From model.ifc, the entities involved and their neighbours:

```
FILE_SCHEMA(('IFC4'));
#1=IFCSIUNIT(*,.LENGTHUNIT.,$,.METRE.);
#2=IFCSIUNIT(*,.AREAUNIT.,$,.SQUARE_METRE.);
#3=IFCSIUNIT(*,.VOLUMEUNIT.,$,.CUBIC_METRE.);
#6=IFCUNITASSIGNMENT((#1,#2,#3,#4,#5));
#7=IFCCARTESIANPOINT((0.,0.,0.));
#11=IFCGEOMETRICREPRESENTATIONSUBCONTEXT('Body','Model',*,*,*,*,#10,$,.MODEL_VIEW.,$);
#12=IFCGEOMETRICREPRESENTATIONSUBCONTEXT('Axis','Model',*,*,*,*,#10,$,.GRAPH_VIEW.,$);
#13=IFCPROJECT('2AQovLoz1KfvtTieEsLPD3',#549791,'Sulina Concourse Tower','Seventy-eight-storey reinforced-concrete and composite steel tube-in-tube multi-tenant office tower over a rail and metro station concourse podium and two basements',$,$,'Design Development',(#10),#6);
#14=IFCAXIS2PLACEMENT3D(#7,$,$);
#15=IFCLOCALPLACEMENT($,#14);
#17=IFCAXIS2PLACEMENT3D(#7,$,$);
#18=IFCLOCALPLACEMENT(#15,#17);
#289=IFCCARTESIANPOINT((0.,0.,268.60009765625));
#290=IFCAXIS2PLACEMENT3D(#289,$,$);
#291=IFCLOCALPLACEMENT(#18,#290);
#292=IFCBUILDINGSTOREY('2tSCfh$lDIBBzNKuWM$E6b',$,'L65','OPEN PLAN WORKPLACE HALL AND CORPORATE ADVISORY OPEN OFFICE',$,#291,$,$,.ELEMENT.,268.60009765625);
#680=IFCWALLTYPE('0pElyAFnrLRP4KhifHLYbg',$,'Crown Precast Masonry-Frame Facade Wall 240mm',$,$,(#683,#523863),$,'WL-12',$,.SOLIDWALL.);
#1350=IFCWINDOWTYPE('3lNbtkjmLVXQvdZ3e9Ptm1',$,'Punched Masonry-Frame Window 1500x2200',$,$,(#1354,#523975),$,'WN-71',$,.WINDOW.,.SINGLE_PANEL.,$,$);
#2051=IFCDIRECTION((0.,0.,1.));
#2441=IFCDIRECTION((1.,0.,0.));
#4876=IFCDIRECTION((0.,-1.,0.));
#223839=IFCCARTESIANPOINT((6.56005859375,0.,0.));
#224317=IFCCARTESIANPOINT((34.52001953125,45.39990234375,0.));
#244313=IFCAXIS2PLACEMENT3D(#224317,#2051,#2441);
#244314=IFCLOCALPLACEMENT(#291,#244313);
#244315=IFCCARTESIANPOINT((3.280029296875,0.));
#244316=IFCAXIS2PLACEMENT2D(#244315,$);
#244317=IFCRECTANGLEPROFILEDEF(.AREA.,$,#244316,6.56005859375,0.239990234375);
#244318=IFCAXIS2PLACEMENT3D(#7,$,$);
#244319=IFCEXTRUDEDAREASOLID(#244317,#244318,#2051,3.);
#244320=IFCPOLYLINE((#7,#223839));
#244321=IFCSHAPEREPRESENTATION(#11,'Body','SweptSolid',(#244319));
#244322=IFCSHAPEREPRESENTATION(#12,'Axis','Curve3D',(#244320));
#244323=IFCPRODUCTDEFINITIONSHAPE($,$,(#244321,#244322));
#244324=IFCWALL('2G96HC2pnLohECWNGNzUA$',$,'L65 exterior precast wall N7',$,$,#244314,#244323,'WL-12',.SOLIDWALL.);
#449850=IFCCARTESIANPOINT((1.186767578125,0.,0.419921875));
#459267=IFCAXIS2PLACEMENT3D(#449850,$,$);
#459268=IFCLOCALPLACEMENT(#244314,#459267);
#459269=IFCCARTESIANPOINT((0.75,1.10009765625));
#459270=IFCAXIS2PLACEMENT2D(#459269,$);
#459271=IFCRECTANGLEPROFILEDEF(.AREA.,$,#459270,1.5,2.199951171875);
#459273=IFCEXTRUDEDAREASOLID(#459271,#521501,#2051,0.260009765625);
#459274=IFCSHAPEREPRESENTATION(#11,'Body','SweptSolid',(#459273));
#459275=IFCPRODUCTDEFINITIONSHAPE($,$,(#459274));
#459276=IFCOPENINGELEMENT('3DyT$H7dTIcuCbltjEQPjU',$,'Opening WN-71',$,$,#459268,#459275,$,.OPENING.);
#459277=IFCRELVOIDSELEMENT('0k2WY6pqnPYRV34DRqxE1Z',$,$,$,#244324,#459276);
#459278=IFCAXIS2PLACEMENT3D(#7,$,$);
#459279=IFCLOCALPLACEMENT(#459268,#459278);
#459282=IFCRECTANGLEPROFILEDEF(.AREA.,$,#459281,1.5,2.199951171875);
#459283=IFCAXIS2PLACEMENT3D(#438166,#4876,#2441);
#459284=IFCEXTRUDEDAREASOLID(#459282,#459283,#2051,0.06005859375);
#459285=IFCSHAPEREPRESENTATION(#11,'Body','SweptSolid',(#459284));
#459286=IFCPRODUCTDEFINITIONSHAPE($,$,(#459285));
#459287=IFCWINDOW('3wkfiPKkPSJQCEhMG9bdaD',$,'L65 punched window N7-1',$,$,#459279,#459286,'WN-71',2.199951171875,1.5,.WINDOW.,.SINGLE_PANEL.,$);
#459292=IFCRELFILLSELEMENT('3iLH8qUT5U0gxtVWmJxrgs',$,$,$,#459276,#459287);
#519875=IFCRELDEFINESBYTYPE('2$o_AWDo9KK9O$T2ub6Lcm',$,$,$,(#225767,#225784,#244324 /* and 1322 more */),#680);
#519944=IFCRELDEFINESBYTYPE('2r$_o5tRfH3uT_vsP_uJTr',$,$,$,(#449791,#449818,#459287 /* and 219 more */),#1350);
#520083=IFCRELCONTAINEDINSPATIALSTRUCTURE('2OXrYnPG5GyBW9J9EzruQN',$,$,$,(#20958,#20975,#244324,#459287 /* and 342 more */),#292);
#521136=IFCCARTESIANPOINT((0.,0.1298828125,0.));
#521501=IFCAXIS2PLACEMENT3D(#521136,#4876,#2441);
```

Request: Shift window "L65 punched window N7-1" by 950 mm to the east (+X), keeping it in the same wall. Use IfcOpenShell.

```python
import ifcopenshell
import ifcopenshell.api.geometry
import ifcopenshell.util.placement

model = ifcopenshell.open("model.ifc")

window = model.by_guid("3wkfiPKkPSJQCEhMG9bdaD")
opening = window.FillsVoids[0].RelatingOpeningElement
wall = opening.VoidsElements[0].RelatingBuildingElement

wall_matrix = ifcopenshell.util.placement.get_local_placement(wall.ObjectPlacement)
shift = wall_matrix[:3, 0] * 0.95
before = ifcopenshell.util.placement.get_local_placement(window.ObjectPlacement)[:3, 3].copy()

# The window is placed relative to its opening, so it follows when the opening moves.
matrix = ifcopenshell.util.placement.get_local_placement(opening.ObjectPlacement)
matrix[:3, 3] += shift
ifcopenshell.api.geometry.edit_object_placement(
    model, product=opening, matrix=matrix, is_si=False, should_transform_children=True
)

after = ifcopenshell.util.placement.get_local_placement(window.ObjectPlacement)[:3, 3]
print("window moved by", (after - before).round(3) + 0.0)

model.write("model-out.ifc")
```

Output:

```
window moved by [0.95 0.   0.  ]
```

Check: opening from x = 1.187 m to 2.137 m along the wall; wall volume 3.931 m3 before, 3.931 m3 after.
